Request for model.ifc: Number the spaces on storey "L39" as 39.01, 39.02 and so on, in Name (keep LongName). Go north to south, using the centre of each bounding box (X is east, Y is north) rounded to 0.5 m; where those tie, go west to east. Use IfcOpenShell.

First a look at what the model holds.

```python
import ifcopenshell
import ifcopenshell.util.element
import ifcopenshell.util.placement

model = ifcopenshell.open("model.ifc")
print(model.schema)
storey = next(s for s in model.by_type("IfcBuildingStorey") if s.Name == "L39")
spaces = [e for e in ifcopenshell.util.element.get_decomposition(storey) if e.is_a("IfcSpace")]
for e in sorted(spaces, key=lambda e: e.id()):
    origin = ifcopenshell.util.placement.get_local_placement(e.ObjectPlacement)[:3, 3]
    print(e.id(), e.Name, e.LongName, origin.round(2) + 0.0, sep=" | ")
```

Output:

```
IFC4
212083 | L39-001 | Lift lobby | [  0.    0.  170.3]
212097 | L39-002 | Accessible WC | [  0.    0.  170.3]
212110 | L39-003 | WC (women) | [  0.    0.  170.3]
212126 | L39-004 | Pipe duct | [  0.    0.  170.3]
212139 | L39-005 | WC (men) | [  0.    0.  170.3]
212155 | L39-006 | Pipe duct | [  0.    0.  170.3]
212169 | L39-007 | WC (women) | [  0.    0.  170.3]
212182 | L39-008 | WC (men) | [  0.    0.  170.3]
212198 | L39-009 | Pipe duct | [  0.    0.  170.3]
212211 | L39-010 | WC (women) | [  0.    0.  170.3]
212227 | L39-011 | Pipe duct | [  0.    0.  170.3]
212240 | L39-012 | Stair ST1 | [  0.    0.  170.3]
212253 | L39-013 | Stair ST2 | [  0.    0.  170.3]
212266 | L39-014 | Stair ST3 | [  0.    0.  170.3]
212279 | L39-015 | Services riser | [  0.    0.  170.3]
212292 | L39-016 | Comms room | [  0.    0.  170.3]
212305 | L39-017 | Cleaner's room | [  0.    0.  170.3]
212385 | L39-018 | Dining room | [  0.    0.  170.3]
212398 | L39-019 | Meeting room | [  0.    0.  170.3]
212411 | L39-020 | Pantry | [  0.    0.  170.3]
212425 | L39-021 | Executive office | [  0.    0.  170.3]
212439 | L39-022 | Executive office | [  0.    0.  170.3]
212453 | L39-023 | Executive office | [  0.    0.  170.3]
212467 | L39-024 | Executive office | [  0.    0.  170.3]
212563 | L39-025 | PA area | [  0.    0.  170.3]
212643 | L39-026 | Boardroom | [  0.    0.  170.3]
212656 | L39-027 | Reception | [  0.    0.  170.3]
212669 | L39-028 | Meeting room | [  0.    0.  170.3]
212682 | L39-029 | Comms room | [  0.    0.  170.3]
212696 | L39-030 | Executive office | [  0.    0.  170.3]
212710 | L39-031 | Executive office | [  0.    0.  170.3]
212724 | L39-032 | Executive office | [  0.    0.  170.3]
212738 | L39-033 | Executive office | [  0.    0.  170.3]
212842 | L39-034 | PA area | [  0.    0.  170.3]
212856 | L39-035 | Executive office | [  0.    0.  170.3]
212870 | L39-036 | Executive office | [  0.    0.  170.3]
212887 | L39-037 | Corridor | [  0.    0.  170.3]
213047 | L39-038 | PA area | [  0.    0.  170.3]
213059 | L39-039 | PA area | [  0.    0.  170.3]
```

```python
import ifcopenshell
import ifcopenshell.geom
import ifcopenshell.util.element
import ifcopenshell.util.shape

model = ifcopenshell.open("model.ifc")
settings = ifcopenshell.geom.settings()
settings.set("use-world-coords", True)


def centre(element):
    shape = ifcopenshell.geom.create_shape(settings, element)
    return ifcopenshell.util.shape.get_bbox_centroid(shape.geometry)


storey = next(s for s in model.by_type("IfcBuildingStorey") if s.Name == "L39")
spaces = [e for e in ifcopenshell.util.element.get_decomposition(storey) if e.is_a("IfcSpace")]

# Insertion points can sit at a corner or the storey origin, so sort by the geometry (in metres).
centres = {e: centre(e) for e in spaces}
spaces.sort(key=lambda e: (-round(centres[e][1] / 0.5), centres[e][0]))

for i, e in enumerate(spaces, start=1):
    number = f"39.{i:02d}"
    e.Name = number
    print(e.id(), number)

model.write("model_rev.ifc")
```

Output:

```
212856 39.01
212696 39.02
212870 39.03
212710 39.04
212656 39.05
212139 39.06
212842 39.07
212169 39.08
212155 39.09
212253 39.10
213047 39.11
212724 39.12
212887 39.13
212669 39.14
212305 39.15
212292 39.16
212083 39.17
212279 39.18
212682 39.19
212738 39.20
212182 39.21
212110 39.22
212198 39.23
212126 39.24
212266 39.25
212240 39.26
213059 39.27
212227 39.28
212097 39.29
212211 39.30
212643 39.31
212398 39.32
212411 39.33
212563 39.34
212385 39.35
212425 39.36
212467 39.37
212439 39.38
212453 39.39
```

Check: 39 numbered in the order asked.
